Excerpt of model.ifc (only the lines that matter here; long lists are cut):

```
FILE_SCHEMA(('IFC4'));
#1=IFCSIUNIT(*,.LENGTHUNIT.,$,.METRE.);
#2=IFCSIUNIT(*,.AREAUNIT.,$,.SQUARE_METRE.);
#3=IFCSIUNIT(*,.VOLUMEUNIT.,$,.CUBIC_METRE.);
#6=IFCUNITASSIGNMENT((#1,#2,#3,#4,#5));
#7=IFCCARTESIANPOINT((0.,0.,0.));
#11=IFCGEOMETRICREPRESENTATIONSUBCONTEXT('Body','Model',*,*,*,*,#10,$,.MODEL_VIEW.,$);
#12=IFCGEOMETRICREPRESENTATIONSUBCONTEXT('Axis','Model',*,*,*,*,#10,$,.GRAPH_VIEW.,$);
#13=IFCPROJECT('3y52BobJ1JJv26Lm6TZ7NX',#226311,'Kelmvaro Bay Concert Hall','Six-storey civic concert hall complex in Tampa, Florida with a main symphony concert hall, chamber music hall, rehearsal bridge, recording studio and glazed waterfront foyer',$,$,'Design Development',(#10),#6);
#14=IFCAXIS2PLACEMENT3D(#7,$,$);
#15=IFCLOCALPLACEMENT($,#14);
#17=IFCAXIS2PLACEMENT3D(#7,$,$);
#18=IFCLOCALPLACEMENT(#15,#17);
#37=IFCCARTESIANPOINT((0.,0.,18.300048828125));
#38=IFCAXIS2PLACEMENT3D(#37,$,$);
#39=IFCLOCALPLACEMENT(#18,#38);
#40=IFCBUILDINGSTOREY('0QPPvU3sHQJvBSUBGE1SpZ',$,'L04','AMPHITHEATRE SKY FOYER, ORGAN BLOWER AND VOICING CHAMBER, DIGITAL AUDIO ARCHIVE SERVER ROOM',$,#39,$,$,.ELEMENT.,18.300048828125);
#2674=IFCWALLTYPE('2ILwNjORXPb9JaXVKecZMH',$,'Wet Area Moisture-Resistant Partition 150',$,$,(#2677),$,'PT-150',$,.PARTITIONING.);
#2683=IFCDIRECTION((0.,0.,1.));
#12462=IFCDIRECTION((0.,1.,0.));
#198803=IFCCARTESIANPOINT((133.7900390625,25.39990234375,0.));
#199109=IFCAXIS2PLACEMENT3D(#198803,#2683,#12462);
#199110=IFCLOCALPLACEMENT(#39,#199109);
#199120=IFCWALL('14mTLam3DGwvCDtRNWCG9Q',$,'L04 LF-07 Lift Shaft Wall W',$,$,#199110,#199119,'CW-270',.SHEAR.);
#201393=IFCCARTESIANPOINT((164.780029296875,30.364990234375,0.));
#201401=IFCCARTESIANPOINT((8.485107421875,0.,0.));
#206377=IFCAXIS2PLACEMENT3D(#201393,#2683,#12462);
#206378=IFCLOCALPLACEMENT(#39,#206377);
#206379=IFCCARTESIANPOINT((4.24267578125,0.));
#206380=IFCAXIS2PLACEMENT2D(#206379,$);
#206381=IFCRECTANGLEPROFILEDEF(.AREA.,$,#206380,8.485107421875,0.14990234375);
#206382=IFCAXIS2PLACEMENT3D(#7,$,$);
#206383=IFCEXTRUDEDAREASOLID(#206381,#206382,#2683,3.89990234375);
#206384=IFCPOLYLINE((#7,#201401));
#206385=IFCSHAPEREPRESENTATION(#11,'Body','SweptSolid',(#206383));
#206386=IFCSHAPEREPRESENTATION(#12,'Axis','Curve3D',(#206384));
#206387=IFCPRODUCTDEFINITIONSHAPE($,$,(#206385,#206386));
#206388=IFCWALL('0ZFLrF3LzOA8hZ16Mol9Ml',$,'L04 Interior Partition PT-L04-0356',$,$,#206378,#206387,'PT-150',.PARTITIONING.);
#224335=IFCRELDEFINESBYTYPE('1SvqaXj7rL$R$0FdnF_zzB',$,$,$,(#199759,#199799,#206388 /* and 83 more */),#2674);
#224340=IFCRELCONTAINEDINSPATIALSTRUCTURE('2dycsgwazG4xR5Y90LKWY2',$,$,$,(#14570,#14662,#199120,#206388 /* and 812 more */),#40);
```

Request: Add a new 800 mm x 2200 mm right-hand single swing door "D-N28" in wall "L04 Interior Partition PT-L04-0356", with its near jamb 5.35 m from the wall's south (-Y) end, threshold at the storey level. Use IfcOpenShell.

```python
import numpy as np
import ifcopenshell
import ifcopenshell.api.feature
import ifcopenshell.api.geometry
import ifcopenshell.api.root
import ifcopenshell.api.spatial
import ifcopenshell.geom
import ifcopenshell.util.element
import ifcopenshell.util.placement
import ifcopenshell.util.representation
import ifcopenshell.util.shape
import ifcopenshell.util.unit

model = ifcopenshell.open("model.ifc")
unit_scale = ifcopenshell.util.unit.calculate_unit_scale(model)
settings = ifcopenshell.geom.settings()


def volume(element):
    """Net volume in cubic metres, openings subtracted."""
    shape = ifcopenshell.geom.create_shape(settings, element)
    return ifcopenshell.util.shape.get_volume(shape.geometry)


wall = model.by_guid("0ZFLrF3LzOA8hZ16Mol9Ml")
storey = ifcopenshell.util.element.get_container(wall, ifc_class="IfcBuildingStorey")
context = ifcopenshell.util.representation.get_context(model, "Model", "Body", "MODEL_VIEW")
before = volume(wall)

width, height, from_end, sill = 0.8, 2.2, 5.35, 0.0  # metres

# The wall runs along its own X axis, and the end named is its -X end.
wall_shape = ifcopenshell.geom.create_shape(settings, wall)
x, y, z = ifcopenshell.util.shape.get_vertices(wall_shape.geometry).T
start = x.min() + from_end
face, thickness = float(y.min()), float(y.max() - y.min())
wall_matrix = ifcopenshell.util.placement.get_local_placement(wall.ObjectPlacement)
level = ifcopenshell.util.placement.get_local_placement(storey.ObjectPlacement)[2, 3]


def in_wall(x, y):
    """Placement at x, y metres in the wall's axes, at sill height."""
    matrix = wall_matrix.copy()
    matrix[:, 3] = wall_matrix @ np.array([x / unit_scale, y / unit_scale, 0.0, 1.0])
    matrix[2, 3] = level + sill / unit_scale
    return matrix


# Opening: a box that overshoots both wall faces by 50 mm.
opening = ifcopenshell.api.root.create_entity(model, ifc_class="IfcOpeningElement", predefined_type="OPENING")
box = ifcopenshell.api.geometry.add_wall_representation(
    model, context=context, length=width, height=height, thickness=thickness + 0.1
)
ifcopenshell.api.geometry.assign_representation(model, product=opening, representation=box)
ifcopenshell.api.geometry.edit_object_placement(model, product=opening, matrix=in_wall(start, face - 0.05), is_si=False)
ifcopenshell.api.feature.add_feature(model, feature=opening, element=wall)

door = ifcopenshell.api.root.create_entity(model, ifc_class="IfcDoor", name="D-N28", predefined_type="DOOR")
door.OverallWidth, door.OverallHeight = width / unit_scale, height / unit_scale
door.OperationType = "SINGLE_SWING_RIGHT"
body = ifcopenshell.api.geometry.add_door_representation(
    model,
    context=context,
    overall_width=door.OverallWidth,
    overall_height=door.OverallHeight,
    operation_type="SINGLE_SWING_RIGHT",
    lining_properties={"LiningDepth": thickness / unit_scale, "ThresholdDepth": thickness / unit_scale},
)
ifcopenshell.api.geometry.assign_representation(model, product=door, representation=body)
ifcopenshell.api.spatial.assign_container(model, products=[door], relating_structure=storey)
ifcopenshell.api.feature.add_filling(model, opening=opening, element=door)

# The lining spans the wall, so the door starts at the wall face.
ifcopenshell.api.geometry.edit_object_placement(model, product=door, matrix=in_wall(start, face), is_si=False)

after = volume(wall)

print(f"wall volume {before:.3f} -> {after:.3f} m3")

model.write("model_rev.ifc")
```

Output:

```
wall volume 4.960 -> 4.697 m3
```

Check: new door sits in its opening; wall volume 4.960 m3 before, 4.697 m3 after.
